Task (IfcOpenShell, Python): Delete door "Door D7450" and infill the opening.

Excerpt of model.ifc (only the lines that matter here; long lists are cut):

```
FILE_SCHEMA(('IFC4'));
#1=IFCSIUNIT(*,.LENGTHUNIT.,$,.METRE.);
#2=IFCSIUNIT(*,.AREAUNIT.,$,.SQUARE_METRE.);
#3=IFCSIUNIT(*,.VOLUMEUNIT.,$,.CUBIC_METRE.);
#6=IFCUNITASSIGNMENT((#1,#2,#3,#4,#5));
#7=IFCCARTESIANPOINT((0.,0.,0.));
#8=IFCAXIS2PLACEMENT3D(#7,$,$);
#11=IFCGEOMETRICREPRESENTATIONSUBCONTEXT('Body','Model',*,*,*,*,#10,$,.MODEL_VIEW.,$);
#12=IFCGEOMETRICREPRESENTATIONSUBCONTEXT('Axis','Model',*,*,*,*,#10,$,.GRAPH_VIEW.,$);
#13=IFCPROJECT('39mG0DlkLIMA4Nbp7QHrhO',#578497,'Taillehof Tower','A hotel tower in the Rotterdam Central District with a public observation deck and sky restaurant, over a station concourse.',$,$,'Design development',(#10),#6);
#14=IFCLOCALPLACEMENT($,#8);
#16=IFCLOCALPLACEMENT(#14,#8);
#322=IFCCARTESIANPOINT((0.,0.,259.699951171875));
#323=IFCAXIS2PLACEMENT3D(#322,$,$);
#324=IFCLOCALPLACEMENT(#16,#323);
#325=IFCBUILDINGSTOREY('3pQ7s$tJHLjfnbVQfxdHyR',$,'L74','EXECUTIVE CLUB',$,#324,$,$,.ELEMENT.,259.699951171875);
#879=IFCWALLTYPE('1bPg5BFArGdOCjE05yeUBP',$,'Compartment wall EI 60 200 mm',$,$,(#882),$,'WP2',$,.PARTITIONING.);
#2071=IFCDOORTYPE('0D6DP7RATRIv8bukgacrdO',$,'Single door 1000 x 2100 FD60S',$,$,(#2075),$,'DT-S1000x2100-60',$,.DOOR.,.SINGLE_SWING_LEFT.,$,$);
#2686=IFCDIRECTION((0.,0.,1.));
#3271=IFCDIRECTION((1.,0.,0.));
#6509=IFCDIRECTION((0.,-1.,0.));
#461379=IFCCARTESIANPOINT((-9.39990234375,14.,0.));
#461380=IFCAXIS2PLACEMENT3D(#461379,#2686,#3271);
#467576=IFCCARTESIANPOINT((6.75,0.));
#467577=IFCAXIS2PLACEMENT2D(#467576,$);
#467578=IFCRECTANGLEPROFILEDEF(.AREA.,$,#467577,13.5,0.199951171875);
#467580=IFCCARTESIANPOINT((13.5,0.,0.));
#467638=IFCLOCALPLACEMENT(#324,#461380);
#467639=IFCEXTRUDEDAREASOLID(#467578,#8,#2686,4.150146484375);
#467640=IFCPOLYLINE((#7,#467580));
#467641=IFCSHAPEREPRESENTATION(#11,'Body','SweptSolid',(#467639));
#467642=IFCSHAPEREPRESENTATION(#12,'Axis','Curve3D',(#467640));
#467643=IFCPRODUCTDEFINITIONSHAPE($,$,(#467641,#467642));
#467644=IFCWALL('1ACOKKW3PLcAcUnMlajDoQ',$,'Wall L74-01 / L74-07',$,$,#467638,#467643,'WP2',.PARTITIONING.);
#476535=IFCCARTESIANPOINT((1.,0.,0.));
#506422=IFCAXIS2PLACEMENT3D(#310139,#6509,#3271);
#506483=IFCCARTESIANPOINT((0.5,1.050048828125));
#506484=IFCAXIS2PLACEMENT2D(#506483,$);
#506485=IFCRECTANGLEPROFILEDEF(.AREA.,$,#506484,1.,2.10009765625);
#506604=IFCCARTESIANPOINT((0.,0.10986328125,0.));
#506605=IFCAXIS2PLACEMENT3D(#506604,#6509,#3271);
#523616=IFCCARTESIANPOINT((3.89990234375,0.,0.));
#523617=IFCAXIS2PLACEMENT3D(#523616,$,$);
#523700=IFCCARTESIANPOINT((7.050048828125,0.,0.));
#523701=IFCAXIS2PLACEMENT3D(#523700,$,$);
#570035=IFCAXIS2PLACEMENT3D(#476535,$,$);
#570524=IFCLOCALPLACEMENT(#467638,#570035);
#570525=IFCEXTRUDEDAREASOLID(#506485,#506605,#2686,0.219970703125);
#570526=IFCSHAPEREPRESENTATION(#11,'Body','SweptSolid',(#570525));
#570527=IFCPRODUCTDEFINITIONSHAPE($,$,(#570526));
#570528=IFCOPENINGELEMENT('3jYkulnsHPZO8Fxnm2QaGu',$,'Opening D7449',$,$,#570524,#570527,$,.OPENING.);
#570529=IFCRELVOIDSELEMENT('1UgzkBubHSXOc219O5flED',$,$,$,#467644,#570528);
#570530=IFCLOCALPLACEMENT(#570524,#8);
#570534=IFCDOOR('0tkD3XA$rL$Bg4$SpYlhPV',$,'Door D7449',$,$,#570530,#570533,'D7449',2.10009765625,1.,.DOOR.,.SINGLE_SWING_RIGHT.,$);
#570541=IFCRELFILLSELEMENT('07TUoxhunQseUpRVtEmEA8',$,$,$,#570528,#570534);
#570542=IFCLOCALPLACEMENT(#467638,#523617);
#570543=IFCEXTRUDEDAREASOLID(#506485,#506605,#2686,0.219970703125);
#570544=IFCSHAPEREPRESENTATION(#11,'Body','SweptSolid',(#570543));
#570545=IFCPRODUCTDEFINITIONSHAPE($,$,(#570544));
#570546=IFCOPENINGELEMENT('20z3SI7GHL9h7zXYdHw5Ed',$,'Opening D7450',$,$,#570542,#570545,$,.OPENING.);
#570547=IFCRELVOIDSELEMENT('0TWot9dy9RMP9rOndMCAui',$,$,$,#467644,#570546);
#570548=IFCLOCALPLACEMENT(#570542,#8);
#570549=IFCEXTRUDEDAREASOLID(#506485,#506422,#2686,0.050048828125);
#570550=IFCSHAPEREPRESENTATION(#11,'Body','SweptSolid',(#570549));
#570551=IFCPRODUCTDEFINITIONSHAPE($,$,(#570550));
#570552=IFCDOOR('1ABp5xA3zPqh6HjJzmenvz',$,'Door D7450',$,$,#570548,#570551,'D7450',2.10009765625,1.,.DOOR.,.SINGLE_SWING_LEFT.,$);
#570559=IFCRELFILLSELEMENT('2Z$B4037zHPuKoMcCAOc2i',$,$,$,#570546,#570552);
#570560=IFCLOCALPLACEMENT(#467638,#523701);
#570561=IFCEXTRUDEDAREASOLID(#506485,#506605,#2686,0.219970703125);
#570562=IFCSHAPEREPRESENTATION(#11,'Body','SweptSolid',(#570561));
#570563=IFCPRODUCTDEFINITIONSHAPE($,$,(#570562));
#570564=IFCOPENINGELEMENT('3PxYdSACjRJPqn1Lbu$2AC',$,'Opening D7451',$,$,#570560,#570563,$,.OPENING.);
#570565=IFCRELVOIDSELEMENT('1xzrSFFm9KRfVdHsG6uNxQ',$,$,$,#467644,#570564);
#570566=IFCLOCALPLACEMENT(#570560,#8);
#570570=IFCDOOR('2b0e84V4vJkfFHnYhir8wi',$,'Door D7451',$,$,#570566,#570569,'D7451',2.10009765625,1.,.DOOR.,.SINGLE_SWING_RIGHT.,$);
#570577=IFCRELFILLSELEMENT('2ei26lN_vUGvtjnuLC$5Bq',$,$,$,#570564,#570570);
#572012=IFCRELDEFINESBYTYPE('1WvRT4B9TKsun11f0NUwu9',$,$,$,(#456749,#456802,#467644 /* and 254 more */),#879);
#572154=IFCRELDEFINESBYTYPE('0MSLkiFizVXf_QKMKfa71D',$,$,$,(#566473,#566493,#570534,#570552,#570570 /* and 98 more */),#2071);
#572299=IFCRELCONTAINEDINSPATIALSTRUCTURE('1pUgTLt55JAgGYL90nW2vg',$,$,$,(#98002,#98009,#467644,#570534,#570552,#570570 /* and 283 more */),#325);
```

```python
import ifcopenshell
import ifcopenshell.api.feature
import ifcopenshell.api.root
import ifcopenshell.geom
import ifcopenshell.util.shape

model = ifcopenshell.open("model.ifc")
settings = ifcopenshell.geom.settings()


def volume(element):
    """Net volume in cubic metres, openings subtracted."""
    shape = ifcopenshell.geom.create_shape(settings, element)
    return ifcopenshell.util.shape.get_volume(shape.geometry)


door = model.by_guid("1ABp5xA3zPqh6HjJzmenvz")
opening = door.FillsVoids[0].RelatingOpeningElement
wall = opening.VoidsElements[0].RelatingBuildingElement
before = volume(wall)

ifcopenshell.api.root.remove_product(model, product=door)
ifcopenshell.api.feature.remove_feature(model, feature=opening)

after = volume(wall)

print(f"wall volume {before:.3f} -> {after:.3f} m3")

model.write("model_rev.ifc")
```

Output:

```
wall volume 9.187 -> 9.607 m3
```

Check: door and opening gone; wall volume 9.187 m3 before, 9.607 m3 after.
